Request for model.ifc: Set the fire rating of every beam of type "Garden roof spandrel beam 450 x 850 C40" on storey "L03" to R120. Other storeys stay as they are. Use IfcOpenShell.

First a look at what the model holds.

```python
import ifcopenshell
import ifcopenshell.util.element

model = ifcopenshell.open("model.ifc")
print(model.schema)
storey = next(s for s in model.by_type("IfcBuildingStorey") if s.Name == "L03")
beams = [e for e in ifcopenshell.util.element.get_decomposition(storey) if e.is_a("IfcBeam")]
seen = {}
for e in beams:
    element_type = ifcopenshell.util.element.get_type(e)
    key = (element_type.Name if element_type != e and element_type else None, ifcopenshell.util.element.get_pset(e, "Pset_BeamCommon", "FireRating"))
    seen[key] = seen.get(key, 0) + 1
for (name, value), count in sorted(seen.items(), key=str):
    print(count, "x", name, "|", value)
```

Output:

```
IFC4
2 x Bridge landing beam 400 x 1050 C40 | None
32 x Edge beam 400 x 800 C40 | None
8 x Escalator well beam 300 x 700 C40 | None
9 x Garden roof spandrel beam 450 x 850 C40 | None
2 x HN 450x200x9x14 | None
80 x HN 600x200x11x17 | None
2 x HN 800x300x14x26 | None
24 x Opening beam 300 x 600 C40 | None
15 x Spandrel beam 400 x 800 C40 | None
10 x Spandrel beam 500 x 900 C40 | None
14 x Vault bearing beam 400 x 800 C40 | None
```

```python
import ifcopenshell
import ifcopenshell.api.pset
import ifcopenshell.util.element

model = ifcopenshell.open("model.ifc")

storey = next(s for s in model.by_type("IfcBuildingStorey") if s.Name == "L03")
beams = [e for e in ifcopenshell.util.element.get_decomposition(storey) if e.is_a("IfcBeam")]

count = 0
for e in beams:
    element_type = ifcopenshell.util.element.get_type(e)
    if element_type in (None, e) or element_type.Name != "Garden roof spandrel beam 450 x 850 C40":
        continue
    # add_pset returns the element's existing set when there is one.
    pset = ifcopenshell.api.pset.add_pset(model, product=e, name="Pset_BeamCommon")
    ifcopenshell.api.pset.edit_pset(model, pset=pset, properties={"FireRating": "R120"})
    count += 1

print(count, "beams updated")

model.write("model_v2.ifc")
```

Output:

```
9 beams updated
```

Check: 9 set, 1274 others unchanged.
